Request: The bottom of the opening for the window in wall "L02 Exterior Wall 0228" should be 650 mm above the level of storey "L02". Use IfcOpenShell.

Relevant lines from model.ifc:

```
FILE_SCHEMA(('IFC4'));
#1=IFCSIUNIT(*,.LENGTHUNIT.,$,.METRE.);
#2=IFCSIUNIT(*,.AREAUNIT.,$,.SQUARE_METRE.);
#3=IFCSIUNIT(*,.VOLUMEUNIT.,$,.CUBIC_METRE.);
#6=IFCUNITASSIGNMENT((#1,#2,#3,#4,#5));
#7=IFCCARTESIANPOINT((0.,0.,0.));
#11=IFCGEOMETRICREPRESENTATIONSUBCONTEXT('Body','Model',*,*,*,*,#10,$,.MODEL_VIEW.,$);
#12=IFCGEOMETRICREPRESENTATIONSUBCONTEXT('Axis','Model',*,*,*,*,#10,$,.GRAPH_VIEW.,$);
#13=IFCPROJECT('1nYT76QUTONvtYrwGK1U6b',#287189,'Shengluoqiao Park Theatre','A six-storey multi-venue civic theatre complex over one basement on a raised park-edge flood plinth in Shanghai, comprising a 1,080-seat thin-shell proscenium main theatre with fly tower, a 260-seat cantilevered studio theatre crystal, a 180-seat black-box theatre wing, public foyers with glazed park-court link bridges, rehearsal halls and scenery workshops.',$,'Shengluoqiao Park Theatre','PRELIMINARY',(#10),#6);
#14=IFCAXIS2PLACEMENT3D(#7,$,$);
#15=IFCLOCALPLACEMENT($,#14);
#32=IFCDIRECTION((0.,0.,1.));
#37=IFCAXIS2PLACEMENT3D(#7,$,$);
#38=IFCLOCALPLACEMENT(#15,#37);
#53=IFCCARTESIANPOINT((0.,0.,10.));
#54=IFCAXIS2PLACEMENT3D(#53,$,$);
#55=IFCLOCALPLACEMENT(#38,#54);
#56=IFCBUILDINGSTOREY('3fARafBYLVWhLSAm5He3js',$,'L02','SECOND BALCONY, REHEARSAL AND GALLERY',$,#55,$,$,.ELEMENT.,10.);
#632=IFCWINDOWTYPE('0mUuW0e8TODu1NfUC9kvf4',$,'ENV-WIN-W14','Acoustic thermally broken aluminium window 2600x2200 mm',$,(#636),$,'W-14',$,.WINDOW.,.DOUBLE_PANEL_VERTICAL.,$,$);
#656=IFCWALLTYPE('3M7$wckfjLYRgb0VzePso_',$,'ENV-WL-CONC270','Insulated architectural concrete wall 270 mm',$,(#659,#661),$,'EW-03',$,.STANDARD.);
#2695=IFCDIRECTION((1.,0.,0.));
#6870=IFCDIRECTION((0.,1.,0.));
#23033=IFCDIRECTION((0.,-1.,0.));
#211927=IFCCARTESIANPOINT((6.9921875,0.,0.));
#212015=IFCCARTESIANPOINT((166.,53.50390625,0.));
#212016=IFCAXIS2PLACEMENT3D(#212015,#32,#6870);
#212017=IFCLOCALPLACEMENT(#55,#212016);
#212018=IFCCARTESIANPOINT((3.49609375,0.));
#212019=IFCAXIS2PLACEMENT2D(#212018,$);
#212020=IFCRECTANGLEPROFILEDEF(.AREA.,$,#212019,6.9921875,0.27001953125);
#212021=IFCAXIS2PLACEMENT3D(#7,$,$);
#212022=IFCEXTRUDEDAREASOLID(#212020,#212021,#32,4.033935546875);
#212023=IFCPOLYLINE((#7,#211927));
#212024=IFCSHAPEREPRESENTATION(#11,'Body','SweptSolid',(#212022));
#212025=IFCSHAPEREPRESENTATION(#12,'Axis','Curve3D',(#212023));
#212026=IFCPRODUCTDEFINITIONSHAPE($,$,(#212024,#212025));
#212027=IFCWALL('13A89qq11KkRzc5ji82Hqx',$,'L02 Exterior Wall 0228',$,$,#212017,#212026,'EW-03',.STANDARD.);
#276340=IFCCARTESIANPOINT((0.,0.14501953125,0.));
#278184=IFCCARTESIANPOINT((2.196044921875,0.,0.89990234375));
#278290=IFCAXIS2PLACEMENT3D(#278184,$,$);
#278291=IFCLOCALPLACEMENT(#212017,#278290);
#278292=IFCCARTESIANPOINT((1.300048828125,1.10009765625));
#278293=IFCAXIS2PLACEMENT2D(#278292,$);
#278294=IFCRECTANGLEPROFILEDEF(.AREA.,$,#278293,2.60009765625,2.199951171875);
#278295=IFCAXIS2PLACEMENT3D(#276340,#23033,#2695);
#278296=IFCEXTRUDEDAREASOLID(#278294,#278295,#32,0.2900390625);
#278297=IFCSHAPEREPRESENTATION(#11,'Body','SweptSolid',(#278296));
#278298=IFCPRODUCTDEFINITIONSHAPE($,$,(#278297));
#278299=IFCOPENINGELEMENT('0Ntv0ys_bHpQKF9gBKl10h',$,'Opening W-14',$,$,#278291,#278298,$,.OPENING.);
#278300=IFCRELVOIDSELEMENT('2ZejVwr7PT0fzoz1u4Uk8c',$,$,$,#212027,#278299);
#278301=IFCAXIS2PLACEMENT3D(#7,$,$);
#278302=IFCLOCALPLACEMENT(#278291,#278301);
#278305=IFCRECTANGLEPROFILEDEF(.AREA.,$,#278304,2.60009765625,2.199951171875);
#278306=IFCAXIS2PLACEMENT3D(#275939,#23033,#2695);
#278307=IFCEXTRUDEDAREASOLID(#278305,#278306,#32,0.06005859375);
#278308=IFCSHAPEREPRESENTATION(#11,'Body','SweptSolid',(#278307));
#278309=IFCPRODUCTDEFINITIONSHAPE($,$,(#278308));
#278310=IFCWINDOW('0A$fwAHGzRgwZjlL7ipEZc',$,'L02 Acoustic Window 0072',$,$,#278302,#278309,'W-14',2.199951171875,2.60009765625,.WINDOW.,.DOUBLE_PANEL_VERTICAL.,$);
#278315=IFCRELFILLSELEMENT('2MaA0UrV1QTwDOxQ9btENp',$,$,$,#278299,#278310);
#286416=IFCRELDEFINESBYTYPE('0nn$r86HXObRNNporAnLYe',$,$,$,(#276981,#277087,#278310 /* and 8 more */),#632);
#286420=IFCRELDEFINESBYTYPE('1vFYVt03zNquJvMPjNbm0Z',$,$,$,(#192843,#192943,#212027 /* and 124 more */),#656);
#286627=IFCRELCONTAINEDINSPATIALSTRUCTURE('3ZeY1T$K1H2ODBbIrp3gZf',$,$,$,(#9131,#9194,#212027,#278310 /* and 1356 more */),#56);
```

```python
import numpy as np
import ifcopenshell
import ifcopenshell.api.geometry
import ifcopenshell.geom
import ifcopenshell.util.element
import ifcopenshell.util.placement
import ifcopenshell.util.shape
import ifcopenshell.util.unit

model = ifcopenshell.open("model.ifc")
unit_scale = ifcopenshell.util.unit.calculate_unit_scale(model)

window = model.by_guid("0A$fwAHGzRgwZjlL7ipEZc")
opening = window.FillsVoids[0].RelatingOpeningElement
storey = ifcopenshell.util.element.get_container(window, ifc_class="IfcBuildingStorey")
level = ifcopenshell.util.placement.get_local_placement(storey.ObjectPlacement)[2, 3]

# The opening's origin need not be at the sill, so measure its lowest point.
shape = ifcopenshell.geom.create_shape(ifcopenshell.geom.settings(), opening)
bottom = ifcopenshell.util.shape.get_shape_bottom_elevation(shape, shape.geometry) / unit_scale
dz = level + 0.65 / unit_scale - bottom

shift = np.array([0.0, 0.0, dz])
# The window is placed relative to its opening, so it follows when the opening moves.
matrix = ifcopenshell.util.placement.get_local_placement(opening.ObjectPlacement)
matrix[:3, 3] += shift
ifcopenshell.api.geometry.edit_object_placement(
    model, product=opening, matrix=matrix, is_si=False, should_transform_children=True
)

print(f"moved by {dz * unit_scale:+.3f} m")

model.write("model_updated.ifc")
```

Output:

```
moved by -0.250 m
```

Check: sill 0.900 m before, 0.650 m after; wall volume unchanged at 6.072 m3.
